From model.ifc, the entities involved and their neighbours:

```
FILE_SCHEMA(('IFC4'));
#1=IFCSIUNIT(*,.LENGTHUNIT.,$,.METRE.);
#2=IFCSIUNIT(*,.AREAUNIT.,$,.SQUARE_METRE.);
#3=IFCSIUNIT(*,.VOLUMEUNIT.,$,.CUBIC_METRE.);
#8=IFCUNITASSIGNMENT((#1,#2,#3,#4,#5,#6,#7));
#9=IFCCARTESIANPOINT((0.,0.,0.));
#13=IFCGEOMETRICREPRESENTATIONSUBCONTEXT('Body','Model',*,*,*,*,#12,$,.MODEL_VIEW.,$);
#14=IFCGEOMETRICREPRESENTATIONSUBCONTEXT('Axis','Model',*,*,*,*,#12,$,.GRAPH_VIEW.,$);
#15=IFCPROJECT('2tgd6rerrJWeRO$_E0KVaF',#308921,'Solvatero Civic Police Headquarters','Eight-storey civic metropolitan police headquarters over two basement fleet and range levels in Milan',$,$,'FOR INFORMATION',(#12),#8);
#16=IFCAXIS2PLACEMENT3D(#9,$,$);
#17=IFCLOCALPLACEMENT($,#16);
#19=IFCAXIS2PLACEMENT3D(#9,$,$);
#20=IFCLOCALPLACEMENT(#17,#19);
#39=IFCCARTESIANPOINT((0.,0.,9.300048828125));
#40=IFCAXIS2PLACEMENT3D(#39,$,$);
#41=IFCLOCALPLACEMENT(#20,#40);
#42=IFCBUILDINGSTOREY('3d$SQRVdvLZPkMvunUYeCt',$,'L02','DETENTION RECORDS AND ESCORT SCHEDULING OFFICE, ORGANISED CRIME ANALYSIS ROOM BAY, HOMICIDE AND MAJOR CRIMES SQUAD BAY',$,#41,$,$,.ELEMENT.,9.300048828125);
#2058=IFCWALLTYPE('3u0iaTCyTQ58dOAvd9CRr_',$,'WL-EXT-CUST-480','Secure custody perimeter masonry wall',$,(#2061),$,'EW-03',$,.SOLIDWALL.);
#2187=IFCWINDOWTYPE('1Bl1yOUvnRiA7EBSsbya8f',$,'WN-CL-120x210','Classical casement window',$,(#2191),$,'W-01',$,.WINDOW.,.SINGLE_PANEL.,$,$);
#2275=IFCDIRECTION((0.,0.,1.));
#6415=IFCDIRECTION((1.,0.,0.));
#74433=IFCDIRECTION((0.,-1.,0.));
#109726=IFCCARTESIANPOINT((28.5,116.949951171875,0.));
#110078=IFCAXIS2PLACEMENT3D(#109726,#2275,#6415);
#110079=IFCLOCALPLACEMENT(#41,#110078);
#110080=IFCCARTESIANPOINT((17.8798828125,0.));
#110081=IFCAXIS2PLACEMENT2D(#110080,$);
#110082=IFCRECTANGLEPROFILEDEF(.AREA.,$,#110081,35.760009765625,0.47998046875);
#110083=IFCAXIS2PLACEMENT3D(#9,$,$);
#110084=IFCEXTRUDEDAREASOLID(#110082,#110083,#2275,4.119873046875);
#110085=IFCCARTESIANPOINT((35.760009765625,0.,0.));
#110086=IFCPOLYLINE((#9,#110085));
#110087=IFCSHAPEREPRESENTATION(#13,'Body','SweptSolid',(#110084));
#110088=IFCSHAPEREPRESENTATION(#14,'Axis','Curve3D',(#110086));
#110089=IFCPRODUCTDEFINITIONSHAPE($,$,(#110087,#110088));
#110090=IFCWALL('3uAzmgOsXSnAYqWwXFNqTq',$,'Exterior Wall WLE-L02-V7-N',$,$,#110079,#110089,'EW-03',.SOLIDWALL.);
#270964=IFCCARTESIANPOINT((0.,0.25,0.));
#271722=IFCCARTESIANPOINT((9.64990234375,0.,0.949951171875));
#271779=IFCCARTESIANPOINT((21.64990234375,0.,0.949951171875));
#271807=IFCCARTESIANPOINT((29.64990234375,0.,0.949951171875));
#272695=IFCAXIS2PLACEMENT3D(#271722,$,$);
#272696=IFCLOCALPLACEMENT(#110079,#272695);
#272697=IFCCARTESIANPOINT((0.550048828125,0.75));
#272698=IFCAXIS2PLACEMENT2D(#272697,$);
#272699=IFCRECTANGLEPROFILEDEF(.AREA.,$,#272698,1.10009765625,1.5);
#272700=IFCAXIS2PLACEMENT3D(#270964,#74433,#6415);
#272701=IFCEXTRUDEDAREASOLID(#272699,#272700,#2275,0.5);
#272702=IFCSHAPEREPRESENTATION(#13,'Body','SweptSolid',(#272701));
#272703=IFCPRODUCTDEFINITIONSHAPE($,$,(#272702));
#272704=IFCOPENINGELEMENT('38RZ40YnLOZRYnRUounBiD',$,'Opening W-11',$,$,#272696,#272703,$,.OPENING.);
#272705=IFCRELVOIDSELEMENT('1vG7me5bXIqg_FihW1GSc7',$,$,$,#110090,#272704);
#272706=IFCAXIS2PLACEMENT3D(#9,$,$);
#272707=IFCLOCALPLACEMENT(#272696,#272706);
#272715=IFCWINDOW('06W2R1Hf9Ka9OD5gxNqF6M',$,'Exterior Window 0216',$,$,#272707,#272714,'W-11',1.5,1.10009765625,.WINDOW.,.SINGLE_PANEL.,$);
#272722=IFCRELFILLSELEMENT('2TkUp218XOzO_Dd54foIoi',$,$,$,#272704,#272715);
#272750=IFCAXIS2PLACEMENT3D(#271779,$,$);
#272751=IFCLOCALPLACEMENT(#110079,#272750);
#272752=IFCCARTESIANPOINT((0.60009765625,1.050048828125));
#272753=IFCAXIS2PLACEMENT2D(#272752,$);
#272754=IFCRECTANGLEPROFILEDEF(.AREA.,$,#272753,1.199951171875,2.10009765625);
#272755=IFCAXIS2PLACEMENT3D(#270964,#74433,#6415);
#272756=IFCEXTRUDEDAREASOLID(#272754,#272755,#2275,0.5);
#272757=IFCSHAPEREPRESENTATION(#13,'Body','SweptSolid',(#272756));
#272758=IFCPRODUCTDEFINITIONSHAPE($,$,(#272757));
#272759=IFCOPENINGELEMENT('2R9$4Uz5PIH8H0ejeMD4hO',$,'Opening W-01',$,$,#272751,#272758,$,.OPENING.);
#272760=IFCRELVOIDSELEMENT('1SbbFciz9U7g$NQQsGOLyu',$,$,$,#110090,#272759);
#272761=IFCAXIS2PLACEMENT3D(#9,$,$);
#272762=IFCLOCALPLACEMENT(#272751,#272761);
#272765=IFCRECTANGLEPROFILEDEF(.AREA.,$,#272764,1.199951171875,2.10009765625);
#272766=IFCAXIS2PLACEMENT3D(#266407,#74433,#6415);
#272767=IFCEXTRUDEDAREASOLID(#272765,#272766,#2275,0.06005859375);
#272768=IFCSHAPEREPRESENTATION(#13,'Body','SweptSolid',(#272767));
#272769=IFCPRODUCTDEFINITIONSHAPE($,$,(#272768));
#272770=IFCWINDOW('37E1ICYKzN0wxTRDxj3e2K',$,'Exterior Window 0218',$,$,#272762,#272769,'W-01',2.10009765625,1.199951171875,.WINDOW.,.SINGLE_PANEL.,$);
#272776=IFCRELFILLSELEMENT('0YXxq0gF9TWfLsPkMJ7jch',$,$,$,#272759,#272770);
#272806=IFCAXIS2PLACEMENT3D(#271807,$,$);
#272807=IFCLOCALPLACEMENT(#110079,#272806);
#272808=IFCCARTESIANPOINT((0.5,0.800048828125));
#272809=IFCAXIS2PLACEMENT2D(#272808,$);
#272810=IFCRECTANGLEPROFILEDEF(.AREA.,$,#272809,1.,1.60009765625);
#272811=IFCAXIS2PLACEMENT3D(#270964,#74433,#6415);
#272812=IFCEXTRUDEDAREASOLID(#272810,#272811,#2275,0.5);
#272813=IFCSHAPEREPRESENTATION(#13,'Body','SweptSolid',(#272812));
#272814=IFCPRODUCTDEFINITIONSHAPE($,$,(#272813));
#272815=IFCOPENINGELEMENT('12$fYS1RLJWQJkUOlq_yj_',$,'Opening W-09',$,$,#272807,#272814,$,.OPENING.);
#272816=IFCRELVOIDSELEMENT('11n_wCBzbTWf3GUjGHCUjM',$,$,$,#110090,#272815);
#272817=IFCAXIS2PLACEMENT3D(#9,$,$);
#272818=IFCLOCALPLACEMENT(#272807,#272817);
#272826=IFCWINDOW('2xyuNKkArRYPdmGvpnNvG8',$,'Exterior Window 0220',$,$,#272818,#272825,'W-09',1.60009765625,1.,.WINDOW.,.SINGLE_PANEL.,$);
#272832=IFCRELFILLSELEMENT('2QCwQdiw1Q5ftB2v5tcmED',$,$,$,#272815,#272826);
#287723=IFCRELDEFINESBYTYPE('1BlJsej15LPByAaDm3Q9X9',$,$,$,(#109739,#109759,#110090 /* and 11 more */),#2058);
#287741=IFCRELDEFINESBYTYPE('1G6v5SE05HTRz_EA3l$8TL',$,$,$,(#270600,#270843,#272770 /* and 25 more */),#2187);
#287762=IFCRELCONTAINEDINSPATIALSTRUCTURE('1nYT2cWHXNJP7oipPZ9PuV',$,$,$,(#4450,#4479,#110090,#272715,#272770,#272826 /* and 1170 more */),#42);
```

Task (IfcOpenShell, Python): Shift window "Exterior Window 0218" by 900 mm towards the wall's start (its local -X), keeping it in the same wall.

```python
import ifcopenshell
import ifcopenshell.api.geometry
import ifcopenshell.util.placement
import ifcopenshell.util.unit

model = ifcopenshell.open("model.ifc")
unit_scale = ifcopenshell.util.unit.calculate_unit_scale(model)

window = model.by_id(272770)
opening = window.FillsVoids[0].RelatingOpeningElement
wall = opening.VoidsElements[0].RelatingBuildingElement

wall_matrix = ifcopenshell.util.placement.get_local_placement(wall.ObjectPlacement)
shift = wall_matrix[:3, 0] * -0.9 / unit_scale
before = ifcopenshell.util.placement.get_local_placement(window.ObjectPlacement)[:3, 3].copy()

# The window is placed relative to its opening, so it follows when the opening moves.
matrix = ifcopenshell.util.placement.get_local_placement(opening.ObjectPlacement)
matrix[:3, 3] += shift
ifcopenshell.api.geometry.edit_object_placement(
    model, product=opening, matrix=matrix, is_si=False, should_transform_children=True
)

after = ifcopenshell.util.placement.get_local_placement(window.ObjectPlacement)[:3, 3]
print("window moved by", (after - before).round(3) + 0.0)

model.write("model-out.ifc")
```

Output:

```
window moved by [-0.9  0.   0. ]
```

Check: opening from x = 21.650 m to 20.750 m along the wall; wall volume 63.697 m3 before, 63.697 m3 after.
